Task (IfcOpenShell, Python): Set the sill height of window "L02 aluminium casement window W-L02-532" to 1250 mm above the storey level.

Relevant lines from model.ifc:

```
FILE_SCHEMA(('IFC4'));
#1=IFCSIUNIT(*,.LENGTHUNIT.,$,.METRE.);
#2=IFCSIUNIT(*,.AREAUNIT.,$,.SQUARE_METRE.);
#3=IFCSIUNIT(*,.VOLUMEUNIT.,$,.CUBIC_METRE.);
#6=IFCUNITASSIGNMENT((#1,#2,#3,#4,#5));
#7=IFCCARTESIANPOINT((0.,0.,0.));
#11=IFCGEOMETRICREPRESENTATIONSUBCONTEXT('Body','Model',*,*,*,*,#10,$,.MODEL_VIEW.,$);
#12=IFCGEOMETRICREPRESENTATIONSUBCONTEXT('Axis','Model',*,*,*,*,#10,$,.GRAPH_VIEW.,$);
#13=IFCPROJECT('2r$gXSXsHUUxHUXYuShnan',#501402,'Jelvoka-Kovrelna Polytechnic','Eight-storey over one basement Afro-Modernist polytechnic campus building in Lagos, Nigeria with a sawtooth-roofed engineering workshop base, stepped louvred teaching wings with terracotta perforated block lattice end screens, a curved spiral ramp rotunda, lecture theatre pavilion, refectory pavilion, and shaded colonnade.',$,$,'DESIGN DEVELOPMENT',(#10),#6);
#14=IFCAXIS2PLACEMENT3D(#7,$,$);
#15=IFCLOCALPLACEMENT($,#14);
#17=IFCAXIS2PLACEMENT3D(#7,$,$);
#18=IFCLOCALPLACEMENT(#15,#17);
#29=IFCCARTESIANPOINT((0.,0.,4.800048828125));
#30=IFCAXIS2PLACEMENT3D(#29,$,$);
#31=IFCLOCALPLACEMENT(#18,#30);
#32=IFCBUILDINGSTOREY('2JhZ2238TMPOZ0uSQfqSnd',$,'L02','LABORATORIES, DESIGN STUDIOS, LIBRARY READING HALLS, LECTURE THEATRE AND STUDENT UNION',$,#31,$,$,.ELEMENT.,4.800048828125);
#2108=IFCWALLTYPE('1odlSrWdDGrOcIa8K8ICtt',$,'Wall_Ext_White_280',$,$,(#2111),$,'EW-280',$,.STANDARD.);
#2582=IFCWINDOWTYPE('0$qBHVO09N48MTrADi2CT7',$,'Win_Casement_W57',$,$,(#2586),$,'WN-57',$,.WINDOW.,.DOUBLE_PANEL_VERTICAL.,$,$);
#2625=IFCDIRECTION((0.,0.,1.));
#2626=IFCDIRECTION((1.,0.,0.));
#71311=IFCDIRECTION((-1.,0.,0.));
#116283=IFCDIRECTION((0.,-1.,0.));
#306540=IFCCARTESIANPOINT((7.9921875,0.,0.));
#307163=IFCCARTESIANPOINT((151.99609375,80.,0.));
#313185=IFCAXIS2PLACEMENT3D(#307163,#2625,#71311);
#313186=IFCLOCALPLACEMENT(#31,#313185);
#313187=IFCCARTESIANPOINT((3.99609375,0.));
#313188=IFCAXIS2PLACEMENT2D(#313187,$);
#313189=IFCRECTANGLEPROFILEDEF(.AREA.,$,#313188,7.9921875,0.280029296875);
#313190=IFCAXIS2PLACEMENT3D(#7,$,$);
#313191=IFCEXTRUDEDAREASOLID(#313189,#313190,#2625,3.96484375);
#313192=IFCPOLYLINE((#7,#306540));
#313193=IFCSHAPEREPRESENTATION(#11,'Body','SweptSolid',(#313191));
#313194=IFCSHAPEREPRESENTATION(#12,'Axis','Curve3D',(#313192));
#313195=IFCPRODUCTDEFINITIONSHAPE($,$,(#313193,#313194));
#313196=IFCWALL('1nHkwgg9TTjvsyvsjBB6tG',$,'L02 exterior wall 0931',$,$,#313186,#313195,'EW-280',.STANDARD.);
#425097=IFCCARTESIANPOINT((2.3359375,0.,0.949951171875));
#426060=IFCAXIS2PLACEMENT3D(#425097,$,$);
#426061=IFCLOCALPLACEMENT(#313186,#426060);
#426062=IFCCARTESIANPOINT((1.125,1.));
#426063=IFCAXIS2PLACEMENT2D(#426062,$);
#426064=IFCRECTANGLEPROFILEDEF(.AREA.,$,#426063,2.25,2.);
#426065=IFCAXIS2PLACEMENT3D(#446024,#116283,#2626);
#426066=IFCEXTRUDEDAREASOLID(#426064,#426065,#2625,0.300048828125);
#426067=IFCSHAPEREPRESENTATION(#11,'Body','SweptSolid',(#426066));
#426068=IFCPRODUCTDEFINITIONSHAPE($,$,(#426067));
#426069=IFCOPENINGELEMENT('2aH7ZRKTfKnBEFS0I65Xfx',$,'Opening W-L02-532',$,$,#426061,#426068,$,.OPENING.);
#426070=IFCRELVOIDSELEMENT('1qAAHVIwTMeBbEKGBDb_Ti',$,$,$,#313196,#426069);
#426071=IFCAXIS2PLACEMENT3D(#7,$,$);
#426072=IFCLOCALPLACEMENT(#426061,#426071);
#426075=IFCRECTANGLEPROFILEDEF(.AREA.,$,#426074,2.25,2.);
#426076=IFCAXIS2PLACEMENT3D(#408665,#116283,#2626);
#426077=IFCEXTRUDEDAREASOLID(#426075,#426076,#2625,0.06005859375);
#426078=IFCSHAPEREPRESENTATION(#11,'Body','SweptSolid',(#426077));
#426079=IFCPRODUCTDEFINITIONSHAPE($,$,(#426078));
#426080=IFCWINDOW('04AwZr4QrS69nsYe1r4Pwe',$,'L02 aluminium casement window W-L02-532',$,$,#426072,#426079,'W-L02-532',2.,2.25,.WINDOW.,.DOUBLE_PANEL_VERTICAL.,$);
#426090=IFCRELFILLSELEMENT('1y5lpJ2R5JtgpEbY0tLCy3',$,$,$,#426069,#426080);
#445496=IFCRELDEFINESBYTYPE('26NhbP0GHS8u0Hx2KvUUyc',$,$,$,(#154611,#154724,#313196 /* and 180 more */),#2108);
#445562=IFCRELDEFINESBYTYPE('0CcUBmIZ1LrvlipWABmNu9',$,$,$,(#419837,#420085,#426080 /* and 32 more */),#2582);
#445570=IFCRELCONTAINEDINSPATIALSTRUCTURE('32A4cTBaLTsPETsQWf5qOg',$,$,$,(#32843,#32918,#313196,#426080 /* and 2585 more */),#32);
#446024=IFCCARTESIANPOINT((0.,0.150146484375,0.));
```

```python
import numpy as np
import ifcopenshell
import ifcopenshell.api.geometry
import ifcopenshell.geom
import ifcopenshell.util.element
import ifcopenshell.util.placement
import ifcopenshell.util.shape
import ifcopenshell.util.unit

model = ifcopenshell.open("model.ifc")
unit_scale = ifcopenshell.util.unit.calculate_unit_scale(model)

window = model.by_guid("04AwZr4QrS69nsYe1r4Pwe")
opening = window.FillsVoids[0].RelatingOpeningElement
storey = ifcopenshell.util.element.get_container(window, ifc_class="IfcBuildingStorey")
level = ifcopenshell.util.placement.get_local_placement(storey.ObjectPlacement)[2, 3]

# The opening's origin need not be at the sill, so measure its lowest point.
shape = ifcopenshell.geom.create_shape(ifcopenshell.geom.settings(), opening)
bottom = ifcopenshell.util.shape.get_shape_bottom_elevation(shape, shape.geometry) / unit_scale
dz = level + 1.25 / unit_scale - bottom

shift = np.array([0.0, 0.0, dz])
# The window is placed relative to its opening, so it follows when the opening moves.
matrix = ifcopenshell.util.placement.get_local_placement(opening.ObjectPlacement)
matrix[:3, 3] += shift
ifcopenshell.api.geometry.edit_object_placement(
    model, product=opening, matrix=matrix, is_si=False, should_transform_children=True
)

print(f"moved by {dz * unit_scale:+.3f} m")

model.write("model_updated.ifc")
```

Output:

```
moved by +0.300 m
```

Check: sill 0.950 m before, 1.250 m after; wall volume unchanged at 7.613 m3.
